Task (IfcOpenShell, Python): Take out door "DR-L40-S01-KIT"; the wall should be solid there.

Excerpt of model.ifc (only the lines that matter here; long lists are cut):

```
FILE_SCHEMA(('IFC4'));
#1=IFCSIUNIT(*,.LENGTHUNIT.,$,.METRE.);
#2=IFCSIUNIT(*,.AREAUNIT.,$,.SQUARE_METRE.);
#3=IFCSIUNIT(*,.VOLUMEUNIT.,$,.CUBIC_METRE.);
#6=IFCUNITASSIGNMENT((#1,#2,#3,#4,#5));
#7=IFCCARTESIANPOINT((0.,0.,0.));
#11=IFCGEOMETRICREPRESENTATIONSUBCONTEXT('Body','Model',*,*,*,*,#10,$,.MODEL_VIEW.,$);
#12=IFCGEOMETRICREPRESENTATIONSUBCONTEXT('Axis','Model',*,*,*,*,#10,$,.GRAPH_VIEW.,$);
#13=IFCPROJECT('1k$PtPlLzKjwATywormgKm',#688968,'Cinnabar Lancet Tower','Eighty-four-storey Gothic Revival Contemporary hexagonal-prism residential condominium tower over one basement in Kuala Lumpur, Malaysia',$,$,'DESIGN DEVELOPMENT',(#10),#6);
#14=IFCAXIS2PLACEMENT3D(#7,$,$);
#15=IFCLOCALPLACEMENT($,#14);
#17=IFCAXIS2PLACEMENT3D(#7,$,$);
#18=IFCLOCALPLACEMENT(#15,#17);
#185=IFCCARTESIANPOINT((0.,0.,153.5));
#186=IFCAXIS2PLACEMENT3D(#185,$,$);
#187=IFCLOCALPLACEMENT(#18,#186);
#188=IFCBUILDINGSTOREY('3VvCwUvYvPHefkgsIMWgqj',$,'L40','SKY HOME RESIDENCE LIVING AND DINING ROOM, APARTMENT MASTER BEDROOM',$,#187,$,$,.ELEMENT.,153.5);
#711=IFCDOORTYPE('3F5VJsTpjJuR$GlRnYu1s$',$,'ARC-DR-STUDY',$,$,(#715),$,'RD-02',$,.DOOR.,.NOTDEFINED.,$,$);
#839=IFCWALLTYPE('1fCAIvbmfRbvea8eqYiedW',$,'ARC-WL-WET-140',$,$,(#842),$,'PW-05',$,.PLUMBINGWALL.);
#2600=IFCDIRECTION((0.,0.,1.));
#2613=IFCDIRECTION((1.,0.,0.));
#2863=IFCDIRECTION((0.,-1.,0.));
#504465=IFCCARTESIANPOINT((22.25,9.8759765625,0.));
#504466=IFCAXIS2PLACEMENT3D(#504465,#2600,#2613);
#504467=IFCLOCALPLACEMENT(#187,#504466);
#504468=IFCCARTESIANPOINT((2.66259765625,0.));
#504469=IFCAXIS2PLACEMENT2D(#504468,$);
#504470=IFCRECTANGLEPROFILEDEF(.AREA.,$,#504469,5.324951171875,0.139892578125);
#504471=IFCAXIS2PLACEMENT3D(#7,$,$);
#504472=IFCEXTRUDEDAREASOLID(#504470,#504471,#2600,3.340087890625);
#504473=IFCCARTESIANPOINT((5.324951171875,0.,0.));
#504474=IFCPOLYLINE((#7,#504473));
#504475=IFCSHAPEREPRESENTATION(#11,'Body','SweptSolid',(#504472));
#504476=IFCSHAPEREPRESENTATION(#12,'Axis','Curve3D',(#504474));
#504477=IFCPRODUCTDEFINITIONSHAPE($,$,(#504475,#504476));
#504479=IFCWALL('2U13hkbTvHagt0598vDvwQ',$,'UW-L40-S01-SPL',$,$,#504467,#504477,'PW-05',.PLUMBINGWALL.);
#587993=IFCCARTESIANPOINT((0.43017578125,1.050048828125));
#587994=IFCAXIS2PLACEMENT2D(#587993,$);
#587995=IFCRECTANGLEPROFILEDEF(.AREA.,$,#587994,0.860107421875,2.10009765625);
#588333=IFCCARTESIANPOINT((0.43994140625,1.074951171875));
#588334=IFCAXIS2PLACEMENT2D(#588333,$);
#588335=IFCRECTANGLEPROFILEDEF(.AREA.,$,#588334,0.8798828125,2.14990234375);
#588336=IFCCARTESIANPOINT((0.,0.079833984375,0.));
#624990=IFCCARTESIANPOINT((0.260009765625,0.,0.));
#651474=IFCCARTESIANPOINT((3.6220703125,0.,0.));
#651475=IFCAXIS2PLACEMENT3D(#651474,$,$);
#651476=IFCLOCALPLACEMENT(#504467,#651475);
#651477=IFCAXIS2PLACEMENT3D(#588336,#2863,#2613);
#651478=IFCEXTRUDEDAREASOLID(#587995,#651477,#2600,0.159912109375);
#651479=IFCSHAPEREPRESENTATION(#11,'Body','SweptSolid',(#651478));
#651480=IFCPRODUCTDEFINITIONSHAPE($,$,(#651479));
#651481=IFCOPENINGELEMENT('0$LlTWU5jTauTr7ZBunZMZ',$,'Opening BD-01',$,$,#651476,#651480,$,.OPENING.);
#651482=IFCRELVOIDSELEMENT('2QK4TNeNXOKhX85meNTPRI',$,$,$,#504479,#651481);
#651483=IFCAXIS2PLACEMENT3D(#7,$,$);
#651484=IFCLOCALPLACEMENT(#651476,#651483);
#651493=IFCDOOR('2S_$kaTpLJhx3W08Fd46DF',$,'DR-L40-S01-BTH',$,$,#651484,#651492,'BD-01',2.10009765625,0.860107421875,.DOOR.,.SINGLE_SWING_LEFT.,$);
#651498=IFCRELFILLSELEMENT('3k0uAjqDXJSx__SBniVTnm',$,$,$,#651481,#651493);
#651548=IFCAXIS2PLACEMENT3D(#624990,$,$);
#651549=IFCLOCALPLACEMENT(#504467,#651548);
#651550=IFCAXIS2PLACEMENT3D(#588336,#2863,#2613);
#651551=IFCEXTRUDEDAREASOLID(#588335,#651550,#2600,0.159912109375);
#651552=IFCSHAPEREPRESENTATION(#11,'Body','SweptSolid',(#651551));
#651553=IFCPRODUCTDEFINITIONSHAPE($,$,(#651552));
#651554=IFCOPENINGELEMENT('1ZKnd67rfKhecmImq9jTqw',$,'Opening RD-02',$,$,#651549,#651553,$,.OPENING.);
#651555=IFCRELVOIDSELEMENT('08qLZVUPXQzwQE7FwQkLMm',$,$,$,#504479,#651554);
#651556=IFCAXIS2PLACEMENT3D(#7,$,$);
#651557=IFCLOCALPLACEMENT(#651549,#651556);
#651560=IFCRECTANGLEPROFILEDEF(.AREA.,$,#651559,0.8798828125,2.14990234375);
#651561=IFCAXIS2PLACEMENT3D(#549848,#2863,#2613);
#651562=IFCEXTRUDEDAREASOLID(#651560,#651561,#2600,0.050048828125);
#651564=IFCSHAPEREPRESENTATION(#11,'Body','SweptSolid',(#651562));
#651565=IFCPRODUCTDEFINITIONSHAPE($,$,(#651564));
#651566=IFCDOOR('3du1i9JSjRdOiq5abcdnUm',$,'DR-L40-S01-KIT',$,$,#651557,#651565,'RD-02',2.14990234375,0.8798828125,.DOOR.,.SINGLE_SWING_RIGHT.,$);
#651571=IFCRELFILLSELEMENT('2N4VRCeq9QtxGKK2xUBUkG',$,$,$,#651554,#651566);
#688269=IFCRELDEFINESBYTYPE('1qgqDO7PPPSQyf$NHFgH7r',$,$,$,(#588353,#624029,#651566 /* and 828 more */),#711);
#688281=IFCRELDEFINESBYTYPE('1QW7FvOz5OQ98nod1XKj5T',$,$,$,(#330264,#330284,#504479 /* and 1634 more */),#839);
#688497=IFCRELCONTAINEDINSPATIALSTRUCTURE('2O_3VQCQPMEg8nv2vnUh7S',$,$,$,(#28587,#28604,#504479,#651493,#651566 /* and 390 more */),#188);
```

```python
import ifcopenshell
import ifcopenshell.api.feature
import ifcopenshell.api.root
import ifcopenshell.geom
import ifcopenshell.util.shape

model = ifcopenshell.open("model.ifc")
settings = ifcopenshell.geom.settings()


def volume(element):
    """Net volume in cubic metres, openings subtracted."""
    shape = ifcopenshell.geom.create_shape(settings, element)
    return ifcopenshell.util.shape.get_volume(shape.geometry)


door = model.by_guid("3du1i9JSjRdOiq5abcdnUm")
opening = door.FillsVoids[0].RelatingOpeningElement
wall = opening.VoidsElements[0].RelatingBuildingElement
before = volume(wall)

ifcopenshell.api.root.remove_product(model, product=door)
ifcopenshell.api.feature.remove_feature(model, feature=opening)

after = volume(wall)

print(f"wall volume {before:.3f} -> {after:.3f} m3")

model.write("model_rev.ifc")
```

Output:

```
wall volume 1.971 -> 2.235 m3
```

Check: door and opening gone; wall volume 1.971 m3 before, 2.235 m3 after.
